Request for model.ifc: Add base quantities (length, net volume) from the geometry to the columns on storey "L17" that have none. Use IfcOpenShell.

First a look at what the model holds.

```python
import ifcopenshell
import ifcopenshell.util.element
import ifcopenshell.util.unit

model = ifcopenshell.open("model.ifc")
print(model.schema)
for unit_type in ("LENGTHUNIT", "AREAUNIT", "VOLUMEUNIT"):
    print(unit_type, ifcopenshell.util.unit.calculate_unit_scale(model, unit_type))
storey = next(s for s in model.by_type("IfcBuildingStorey") if s.Name == "L17")
columns = [e for e in ifcopenshell.util.element.get_decomposition(storey) if e.is_a("IfcColumn")]
for e in sorted(columns, key=lambda e: e.id()):
    print(e.id(), e.is_a(), e.Name, list(ifcopenshell.util.element.get_psets(e, qtos_only=True)), sep=" | ")
```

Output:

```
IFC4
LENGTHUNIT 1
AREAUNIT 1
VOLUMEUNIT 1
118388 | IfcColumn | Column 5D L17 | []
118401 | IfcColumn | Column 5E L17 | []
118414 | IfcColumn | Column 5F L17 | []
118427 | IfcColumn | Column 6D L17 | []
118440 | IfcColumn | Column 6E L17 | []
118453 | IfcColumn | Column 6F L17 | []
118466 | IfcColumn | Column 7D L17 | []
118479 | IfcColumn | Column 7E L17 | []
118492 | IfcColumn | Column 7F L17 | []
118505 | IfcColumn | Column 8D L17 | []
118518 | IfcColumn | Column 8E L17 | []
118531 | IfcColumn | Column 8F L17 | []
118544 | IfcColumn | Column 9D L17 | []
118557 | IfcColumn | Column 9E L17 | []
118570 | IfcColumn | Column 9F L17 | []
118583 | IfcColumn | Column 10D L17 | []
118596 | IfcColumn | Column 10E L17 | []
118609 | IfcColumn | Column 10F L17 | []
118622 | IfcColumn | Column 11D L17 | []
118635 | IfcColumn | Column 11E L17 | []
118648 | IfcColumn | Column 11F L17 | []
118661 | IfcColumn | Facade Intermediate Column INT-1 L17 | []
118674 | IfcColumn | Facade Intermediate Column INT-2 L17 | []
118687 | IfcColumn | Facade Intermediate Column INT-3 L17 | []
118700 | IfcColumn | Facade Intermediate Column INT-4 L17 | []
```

```python
import ifcopenshell
import ifcopenshell.api.pset
import ifcopenshell.geom
import ifcopenshell.util.element
import ifcopenshell.util.shape
import ifcopenshell.util.unit

model = ifcopenshell.open("model.ifc")
unit_scale = ifcopenshell.util.unit.calculate_unit_scale(model)
volume_scale = ifcopenshell.util.unit.calculate_unit_scale(model, "VOLUMEUNIT")
settings = ifcopenshell.geom.settings()

storey = next(s for s in model.by_type("IfcBuildingStorey") if s.Name == "L17")
columns = [e for e in ifcopenshell.util.element.get_decomposition(storey) if e.is_a("IfcColumn")]

for e in sorted(columns, key=lambda e: e.id()):
    if ifcopenshell.util.element.get_psets(e, qtos_only=True, should_inherit=False):
        continue
    # Geometry comes back in metres, in the element's own axes.
    shape = ifcopenshell.geom.create_shape(settings, e)
    values = {
        "Length": ifcopenshell.util.shape.get_z(shape.geometry) / unit_scale,
        "NetVolume": ifcopenshell.util.shape.get_volume(shape.geometry) / volume_scale,
    }
    qto = ifcopenshell.api.pset.add_qto(model, product=e, name="Qto_ColumnBaseQuantities")
    ifcopenshell.api.pset.edit_qto(model, qto=qto, properties=values)
    print(e.id(), {k: round(v, 3) for k, v in values.items()})

model.write("model_v2.ifc")
```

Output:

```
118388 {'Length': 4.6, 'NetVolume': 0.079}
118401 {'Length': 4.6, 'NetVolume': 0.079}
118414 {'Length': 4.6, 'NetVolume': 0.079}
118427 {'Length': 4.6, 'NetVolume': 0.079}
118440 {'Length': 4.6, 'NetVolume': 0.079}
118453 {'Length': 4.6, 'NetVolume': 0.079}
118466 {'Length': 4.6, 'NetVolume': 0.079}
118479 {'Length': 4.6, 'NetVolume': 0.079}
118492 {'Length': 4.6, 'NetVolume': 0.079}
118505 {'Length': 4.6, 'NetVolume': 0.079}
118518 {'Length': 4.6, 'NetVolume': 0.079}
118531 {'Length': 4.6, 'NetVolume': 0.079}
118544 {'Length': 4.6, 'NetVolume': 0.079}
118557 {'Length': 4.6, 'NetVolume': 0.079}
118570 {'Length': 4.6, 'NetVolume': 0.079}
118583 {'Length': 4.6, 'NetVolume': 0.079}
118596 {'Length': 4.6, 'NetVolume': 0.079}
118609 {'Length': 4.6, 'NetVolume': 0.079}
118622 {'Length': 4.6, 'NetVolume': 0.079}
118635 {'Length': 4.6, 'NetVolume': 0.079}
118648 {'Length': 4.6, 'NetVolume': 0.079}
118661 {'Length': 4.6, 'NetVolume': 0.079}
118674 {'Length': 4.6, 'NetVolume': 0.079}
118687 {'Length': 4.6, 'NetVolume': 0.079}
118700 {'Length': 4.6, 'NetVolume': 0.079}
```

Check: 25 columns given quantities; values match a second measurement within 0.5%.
